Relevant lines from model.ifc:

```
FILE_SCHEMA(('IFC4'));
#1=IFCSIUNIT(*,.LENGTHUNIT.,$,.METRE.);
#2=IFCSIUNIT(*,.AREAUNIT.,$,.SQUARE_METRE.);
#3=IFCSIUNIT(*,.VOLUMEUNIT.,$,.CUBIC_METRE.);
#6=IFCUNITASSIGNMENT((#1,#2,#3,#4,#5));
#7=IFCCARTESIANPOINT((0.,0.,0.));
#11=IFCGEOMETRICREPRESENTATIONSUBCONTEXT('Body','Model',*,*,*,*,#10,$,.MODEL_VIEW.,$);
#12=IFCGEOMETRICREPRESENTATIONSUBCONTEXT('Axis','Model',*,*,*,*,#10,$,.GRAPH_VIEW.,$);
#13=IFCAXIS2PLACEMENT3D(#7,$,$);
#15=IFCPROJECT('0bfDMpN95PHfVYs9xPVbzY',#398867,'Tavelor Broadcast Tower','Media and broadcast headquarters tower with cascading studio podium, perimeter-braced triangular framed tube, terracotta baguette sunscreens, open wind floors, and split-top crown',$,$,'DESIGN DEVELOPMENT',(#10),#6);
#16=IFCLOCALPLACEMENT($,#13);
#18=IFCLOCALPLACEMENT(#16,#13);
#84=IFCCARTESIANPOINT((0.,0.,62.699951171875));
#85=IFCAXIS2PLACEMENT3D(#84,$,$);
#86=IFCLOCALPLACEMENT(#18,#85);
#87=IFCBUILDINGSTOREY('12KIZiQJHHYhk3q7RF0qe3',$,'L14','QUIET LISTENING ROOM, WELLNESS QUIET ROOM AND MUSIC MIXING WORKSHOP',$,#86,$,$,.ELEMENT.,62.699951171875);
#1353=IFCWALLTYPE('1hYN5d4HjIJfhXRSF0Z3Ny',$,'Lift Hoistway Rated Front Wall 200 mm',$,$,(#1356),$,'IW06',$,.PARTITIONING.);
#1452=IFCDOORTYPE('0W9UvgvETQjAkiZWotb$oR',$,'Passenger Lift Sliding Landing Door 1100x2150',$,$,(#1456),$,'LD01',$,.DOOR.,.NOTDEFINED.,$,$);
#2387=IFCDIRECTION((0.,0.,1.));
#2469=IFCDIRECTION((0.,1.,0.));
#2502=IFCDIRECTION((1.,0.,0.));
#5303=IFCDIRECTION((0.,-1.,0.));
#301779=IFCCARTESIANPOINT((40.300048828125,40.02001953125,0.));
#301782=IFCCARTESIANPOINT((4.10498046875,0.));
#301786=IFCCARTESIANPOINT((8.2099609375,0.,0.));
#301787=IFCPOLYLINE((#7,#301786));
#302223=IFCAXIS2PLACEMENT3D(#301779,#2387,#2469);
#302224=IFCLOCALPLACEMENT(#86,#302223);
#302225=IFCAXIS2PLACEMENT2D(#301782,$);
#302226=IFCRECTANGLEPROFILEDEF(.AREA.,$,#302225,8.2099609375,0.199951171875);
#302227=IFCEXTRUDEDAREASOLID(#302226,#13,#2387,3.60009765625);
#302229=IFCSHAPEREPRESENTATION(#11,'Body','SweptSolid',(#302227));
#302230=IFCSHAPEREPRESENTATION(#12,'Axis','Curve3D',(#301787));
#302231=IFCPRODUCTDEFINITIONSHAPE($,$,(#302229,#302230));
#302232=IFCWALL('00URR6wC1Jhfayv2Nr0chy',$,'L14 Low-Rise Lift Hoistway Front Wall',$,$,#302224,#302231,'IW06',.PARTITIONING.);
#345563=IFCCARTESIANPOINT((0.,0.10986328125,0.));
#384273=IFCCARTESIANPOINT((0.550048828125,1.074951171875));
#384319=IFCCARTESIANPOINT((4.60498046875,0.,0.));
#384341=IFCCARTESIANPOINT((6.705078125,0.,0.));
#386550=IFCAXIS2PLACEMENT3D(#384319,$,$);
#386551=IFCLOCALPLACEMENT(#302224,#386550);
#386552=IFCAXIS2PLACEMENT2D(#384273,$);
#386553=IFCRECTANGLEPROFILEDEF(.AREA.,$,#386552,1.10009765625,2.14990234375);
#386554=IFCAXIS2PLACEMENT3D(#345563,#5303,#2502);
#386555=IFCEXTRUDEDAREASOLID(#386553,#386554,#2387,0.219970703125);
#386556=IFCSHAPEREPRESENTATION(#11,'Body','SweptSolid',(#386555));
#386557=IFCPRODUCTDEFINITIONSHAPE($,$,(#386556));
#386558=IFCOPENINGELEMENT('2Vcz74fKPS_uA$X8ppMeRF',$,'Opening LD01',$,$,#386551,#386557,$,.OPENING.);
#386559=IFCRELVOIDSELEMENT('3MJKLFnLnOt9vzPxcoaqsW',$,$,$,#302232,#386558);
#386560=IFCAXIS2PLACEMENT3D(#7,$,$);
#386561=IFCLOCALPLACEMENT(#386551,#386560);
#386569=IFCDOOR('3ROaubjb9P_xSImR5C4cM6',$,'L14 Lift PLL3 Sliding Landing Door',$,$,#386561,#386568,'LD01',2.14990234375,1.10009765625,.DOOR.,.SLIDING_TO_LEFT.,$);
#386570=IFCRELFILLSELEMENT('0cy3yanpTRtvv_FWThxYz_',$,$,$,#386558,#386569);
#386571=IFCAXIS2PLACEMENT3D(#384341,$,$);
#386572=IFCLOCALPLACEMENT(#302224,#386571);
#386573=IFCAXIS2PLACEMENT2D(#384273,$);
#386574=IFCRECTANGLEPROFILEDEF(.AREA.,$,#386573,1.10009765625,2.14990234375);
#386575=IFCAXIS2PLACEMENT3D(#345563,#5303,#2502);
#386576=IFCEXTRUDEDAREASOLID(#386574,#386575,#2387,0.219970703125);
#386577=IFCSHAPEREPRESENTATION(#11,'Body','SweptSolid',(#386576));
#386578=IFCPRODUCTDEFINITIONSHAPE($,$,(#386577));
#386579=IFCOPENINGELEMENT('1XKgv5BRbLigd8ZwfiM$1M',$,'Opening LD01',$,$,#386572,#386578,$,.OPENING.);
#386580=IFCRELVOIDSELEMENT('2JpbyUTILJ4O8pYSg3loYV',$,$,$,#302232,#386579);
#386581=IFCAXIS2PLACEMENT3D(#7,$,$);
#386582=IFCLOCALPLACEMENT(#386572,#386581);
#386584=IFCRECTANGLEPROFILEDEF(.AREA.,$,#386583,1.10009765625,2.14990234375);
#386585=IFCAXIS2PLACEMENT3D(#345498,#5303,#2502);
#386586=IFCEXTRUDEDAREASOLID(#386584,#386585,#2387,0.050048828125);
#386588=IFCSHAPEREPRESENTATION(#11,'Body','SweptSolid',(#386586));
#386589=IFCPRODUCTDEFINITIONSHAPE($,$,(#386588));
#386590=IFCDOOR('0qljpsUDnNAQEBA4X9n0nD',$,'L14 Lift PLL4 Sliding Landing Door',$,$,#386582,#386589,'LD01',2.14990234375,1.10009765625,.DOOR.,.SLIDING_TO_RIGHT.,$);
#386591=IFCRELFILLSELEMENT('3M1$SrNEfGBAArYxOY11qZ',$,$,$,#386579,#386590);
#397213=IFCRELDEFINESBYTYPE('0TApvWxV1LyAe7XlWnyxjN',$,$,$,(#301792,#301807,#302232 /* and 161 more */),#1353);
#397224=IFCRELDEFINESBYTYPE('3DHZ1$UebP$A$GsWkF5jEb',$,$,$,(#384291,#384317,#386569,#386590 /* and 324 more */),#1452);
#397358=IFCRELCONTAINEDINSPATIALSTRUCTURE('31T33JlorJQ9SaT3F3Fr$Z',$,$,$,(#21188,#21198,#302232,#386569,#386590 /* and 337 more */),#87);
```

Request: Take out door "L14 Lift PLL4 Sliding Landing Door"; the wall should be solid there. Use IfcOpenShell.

```python
import ifcopenshell
import ifcopenshell.api.feature
import ifcopenshell.api.root
import ifcopenshell.geom
import ifcopenshell.util.shape

model = ifcopenshell.open("model.ifc")
settings = ifcopenshell.geom.settings()


def volume(element):
    """Net volume in cubic metres, openings subtracted."""
    shape = ifcopenshell.geom.create_shape(settings, element)
    return ifcopenshell.util.shape.get_volume(shape.geometry)


door = model.by_guid("0qljpsUDnNAQEBA4X9n0nD")
opening = door.FillsVoids[0].RelatingOpeningElement
wall = opening.VoidsElements[0].RelatingBuildingElement
before = volume(wall)

ifcopenshell.api.root.remove_product(model, product=door)
ifcopenshell.api.feature.remove_feature(model, feature=opening)

after = volume(wall)

print(f"wall volume {before:.3f} -> {after:.3f} m3")

model.write("model_edited.ifc")
```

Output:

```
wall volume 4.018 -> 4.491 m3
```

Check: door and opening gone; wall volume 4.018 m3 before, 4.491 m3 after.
